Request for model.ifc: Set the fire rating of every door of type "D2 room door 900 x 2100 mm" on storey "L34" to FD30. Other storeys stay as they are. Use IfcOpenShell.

First a look at what the model holds.

```python
import ifcopenshell
import ifcopenshell.util.element

model = ifcopenshell.open("model.ifc")
print(model.schema)
storey = next(s for s in model.by_type("IfcBuildingStorey") if s.Name == "L34")
doors = [e for e in ifcopenshell.util.element.get_decomposition(storey) if e.is_a("IfcDoor")]
seen = {}
for e in doors:
    element_type = ifcopenshell.util.element.get_type(e)
    key = (element_type.Name if element_type != e and element_type else None, ifcopenshell.util.element.get_pset(e, "Pset_DoorCommon", "FireRating"))
    seen[key] = seen.get(key, 0) + 1
for (name, value), count in sorted(seen.items(), key=str):
    print(count, "x", name, "|", value)
```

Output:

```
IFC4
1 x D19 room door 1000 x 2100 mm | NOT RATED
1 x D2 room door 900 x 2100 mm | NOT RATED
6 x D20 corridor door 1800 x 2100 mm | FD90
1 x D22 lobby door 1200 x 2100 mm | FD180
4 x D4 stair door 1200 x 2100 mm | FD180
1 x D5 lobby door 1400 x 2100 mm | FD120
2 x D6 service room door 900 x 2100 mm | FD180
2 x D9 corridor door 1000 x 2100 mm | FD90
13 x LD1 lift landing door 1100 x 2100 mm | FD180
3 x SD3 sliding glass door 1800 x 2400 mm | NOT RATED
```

```python
import ifcopenshell
import ifcopenshell.api.pset
import ifcopenshell.util.element

model = ifcopenshell.open("model.ifc")

storey = next(s for s in model.by_type("IfcBuildingStorey") if s.Name == "L34")
doors = [e for e in ifcopenshell.util.element.get_decomposition(storey) if e.is_a("IfcDoor")]

count = 0
for e in doors:
    element_type = ifcopenshell.util.element.get_type(e)
    if element_type in (None, e) or element_type.Name != "D2 room door 900 x 2100 mm":
        continue
    # add_pset returns the element's existing set when there is one.
    pset = ifcopenshell.api.pset.add_pset(model, product=e, name="Pset_DoorCommon")
    ifcopenshell.api.pset.edit_pset(model, pset=pset, properties={"FireRating": "FD30"})
    count += 1

print(count, "doors updated")

model.write("model_rev.ifc")
```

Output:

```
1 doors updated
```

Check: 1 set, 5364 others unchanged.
